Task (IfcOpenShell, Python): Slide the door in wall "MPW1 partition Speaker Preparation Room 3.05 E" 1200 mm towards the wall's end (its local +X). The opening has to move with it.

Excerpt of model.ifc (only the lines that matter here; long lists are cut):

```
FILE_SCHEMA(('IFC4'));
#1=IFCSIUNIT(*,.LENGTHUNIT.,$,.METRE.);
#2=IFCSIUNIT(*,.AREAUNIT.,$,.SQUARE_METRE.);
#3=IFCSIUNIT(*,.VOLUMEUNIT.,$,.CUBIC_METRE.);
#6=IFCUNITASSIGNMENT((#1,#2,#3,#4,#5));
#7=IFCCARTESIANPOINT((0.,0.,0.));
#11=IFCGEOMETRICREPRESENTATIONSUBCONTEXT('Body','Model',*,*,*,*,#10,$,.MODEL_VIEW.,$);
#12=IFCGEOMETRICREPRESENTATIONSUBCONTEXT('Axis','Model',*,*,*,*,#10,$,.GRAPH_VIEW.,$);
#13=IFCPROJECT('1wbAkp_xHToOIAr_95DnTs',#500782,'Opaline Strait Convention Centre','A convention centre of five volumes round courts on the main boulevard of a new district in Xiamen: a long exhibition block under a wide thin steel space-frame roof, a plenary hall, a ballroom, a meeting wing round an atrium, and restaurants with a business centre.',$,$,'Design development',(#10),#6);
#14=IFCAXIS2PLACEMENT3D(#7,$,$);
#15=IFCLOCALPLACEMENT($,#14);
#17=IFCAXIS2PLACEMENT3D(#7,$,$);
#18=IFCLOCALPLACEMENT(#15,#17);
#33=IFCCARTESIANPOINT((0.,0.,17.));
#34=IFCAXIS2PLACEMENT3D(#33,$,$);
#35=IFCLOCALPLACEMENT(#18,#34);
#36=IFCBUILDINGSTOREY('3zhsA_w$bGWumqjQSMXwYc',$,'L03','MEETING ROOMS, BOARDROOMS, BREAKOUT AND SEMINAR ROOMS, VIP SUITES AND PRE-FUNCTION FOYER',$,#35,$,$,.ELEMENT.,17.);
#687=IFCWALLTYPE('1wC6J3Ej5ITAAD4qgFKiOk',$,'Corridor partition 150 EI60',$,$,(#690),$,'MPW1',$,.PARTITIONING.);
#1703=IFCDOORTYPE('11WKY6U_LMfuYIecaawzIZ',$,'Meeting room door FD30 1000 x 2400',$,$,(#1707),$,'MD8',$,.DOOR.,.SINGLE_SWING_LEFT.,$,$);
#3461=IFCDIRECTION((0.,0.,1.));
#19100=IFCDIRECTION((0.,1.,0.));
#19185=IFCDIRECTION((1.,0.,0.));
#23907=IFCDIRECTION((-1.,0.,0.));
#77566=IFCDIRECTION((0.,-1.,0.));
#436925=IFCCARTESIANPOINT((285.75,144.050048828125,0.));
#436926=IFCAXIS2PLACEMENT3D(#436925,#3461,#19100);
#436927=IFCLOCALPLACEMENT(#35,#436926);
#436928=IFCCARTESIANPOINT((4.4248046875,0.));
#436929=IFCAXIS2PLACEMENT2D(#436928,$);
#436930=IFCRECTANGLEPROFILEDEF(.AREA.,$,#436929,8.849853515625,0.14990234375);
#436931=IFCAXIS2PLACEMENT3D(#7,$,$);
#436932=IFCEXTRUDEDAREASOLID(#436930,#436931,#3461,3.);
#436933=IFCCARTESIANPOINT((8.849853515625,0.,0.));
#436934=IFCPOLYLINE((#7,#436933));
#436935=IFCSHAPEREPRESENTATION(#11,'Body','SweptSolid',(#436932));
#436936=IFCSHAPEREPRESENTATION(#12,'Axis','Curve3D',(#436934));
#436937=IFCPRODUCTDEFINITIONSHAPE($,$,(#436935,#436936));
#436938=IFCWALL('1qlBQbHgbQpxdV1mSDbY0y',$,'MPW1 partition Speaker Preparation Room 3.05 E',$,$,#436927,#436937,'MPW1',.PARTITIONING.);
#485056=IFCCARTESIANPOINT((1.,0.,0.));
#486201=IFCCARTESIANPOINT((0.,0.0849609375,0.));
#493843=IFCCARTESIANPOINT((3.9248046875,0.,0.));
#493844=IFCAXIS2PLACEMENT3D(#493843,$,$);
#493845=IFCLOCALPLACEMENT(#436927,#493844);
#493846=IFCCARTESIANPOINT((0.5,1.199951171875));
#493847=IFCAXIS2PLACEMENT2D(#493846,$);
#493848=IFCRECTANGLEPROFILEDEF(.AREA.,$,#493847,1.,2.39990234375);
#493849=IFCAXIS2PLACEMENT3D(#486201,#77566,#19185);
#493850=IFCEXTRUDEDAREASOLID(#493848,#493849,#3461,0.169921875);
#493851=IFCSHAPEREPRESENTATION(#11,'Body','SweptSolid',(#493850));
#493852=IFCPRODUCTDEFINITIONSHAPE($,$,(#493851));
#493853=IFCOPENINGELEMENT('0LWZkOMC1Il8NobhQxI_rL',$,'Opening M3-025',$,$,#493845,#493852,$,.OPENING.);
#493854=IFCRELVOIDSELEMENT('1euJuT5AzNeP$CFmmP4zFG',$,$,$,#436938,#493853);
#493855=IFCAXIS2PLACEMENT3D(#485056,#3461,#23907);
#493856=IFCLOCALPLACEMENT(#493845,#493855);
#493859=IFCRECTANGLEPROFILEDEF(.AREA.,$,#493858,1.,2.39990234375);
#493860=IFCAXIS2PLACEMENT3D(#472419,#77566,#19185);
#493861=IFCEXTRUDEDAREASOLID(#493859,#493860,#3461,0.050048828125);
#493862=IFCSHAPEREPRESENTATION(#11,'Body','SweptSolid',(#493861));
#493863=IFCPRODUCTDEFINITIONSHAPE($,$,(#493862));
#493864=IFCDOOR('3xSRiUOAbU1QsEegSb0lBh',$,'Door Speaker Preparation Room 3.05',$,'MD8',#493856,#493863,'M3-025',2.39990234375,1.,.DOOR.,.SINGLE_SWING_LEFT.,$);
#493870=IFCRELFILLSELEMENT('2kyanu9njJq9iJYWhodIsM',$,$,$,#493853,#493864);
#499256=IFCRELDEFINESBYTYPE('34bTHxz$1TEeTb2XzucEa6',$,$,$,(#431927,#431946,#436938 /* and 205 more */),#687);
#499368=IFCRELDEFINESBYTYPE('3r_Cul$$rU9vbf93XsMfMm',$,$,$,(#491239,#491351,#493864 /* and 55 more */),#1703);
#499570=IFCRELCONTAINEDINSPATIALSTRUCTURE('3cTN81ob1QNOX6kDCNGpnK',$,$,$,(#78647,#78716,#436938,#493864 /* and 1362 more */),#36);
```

```python
import ifcopenshell
import ifcopenshell.api.geometry
import ifcopenshell.util.placement
import ifcopenshell.util.unit

model = ifcopenshell.open("model.ifc")
unit_scale = ifcopenshell.util.unit.calculate_unit_scale(model)

door = model.by_guid("3xSRiUOAbU1QsEegSb0lBh")
opening = door.FillsVoids[0].RelatingOpeningElement
wall = opening.VoidsElements[0].RelatingBuildingElement

wall_matrix = ifcopenshell.util.placement.get_local_placement(wall.ObjectPlacement)
shift = wall_matrix[:3, 0] * 1.2 / unit_scale
before = ifcopenshell.util.placement.get_local_placement(door.ObjectPlacement)[:3, 3].copy()

# The door is placed relative to its opening, so it follows when the opening moves.
matrix = ifcopenshell.util.placement.get_local_placement(opening.ObjectPlacement)
matrix[:3, 3] += shift
ifcopenshell.api.geometry.edit_object_placement(
    model, product=opening, matrix=matrix, is_si=False, should_transform_children=True
)

after = ifcopenshell.util.placement.get_local_placement(door.ObjectPlacement)[:3, 3]
print("door moved by", (after - before).round(3) + 0.0)

model.write("model-out.ifc")
```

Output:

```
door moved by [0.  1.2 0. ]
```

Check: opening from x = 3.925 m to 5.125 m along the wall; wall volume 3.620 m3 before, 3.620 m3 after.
